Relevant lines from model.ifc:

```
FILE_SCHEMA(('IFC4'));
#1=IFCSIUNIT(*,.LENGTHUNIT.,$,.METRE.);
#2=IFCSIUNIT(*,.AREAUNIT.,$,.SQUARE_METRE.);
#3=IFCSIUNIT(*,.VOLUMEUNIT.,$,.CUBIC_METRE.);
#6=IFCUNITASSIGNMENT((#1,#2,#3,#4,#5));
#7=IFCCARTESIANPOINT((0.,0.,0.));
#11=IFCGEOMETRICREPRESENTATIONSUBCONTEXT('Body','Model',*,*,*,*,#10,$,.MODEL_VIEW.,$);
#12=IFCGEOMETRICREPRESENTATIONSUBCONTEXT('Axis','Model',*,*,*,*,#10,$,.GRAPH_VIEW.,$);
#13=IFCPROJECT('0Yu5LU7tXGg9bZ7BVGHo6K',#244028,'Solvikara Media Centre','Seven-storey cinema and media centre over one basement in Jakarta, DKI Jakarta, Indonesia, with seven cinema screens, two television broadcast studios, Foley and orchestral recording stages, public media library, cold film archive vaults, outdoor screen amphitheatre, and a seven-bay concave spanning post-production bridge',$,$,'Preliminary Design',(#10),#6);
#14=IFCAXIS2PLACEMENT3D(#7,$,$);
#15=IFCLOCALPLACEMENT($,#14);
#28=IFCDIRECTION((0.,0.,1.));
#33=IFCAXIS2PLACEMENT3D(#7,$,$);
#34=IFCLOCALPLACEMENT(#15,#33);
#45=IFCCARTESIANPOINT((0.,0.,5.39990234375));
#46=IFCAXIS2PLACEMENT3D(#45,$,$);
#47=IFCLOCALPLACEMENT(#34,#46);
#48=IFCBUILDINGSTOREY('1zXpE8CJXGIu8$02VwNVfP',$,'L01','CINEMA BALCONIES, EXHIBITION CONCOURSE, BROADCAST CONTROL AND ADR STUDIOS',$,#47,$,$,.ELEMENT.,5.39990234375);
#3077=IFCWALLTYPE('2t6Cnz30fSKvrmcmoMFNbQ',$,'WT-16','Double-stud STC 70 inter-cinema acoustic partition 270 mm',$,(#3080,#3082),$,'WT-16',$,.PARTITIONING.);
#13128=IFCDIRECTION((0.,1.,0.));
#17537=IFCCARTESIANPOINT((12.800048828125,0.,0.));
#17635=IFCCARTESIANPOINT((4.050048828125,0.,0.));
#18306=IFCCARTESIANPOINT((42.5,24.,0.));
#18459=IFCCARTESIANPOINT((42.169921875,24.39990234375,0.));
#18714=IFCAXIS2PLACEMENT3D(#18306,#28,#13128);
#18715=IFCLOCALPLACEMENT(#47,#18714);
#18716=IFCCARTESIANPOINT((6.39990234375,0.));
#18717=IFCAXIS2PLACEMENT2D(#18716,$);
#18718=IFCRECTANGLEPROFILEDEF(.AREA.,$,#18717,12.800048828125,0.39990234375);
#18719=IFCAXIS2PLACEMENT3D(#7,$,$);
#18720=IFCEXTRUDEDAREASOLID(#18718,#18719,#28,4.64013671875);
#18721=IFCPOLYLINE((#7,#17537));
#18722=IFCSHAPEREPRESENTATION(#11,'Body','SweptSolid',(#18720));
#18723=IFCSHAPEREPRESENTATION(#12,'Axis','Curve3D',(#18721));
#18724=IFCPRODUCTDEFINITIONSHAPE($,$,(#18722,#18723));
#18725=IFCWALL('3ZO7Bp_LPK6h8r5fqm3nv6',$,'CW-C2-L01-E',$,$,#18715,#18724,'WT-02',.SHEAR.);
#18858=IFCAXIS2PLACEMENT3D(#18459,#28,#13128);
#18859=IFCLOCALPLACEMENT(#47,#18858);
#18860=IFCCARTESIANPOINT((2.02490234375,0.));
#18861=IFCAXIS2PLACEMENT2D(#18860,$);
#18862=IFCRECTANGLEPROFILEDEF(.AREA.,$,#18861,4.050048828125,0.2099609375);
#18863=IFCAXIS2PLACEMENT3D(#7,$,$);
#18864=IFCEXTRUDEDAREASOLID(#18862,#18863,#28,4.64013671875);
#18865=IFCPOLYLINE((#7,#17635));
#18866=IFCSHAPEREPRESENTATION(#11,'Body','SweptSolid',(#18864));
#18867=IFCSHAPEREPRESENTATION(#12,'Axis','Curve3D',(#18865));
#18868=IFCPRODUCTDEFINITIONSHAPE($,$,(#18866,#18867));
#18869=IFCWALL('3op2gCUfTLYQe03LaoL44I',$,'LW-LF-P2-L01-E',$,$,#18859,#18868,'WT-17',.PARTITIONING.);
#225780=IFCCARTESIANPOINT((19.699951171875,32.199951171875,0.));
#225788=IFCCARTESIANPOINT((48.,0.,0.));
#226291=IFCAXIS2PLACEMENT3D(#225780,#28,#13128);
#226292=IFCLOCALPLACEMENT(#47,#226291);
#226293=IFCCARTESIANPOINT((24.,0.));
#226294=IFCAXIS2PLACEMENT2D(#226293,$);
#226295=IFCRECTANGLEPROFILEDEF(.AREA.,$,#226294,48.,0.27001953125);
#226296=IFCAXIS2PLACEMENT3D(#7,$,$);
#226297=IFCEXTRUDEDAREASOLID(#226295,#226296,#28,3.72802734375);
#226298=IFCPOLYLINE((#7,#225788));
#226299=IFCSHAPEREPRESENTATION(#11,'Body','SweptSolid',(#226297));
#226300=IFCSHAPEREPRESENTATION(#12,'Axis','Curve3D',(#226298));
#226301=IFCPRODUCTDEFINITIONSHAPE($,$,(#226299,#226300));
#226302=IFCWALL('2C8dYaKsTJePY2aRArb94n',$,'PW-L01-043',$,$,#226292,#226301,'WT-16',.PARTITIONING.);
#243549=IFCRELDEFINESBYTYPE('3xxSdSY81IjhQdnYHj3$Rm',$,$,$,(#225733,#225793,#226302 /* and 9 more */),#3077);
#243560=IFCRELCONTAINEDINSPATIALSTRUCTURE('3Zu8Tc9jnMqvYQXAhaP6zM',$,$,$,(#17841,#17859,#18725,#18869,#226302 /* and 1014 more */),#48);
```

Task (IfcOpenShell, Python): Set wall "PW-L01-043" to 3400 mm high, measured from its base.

```python
import ifcopenshell
import ifcopenshell.geom
import ifcopenshell.util.representation
import ifcopenshell.util.shape
import ifcopenshell.util.unit

model = ifcopenshell.open("model.ifc")
unit_scale = ifcopenshell.util.unit.calculate_unit_scale(model)
settings = ifcopenshell.geom.settings()


def volume(element):
    """Net volume in cubic metres, openings subtracted."""
    shape = ifcopenshell.geom.create_shape(settings, element)
    return ifcopenshell.util.shape.get_volume(shape.geometry)


wall = model.by_guid("2C8dYaKsTJePY2aRArb94n")
before = volume(wall)

body = ifcopenshell.util.representation.get_representation(wall, "Model", "Body")
solid = body.Items[0]
old_height = solid.Depth
solid.Depth = 3.4 / unit_scale
after = volume(wall)

print(f"height {old_height:g} -> {solid.Depth:g}, volume {before:.3f} -> {after:.3f} m3")

model.write("model-out.ifc")
```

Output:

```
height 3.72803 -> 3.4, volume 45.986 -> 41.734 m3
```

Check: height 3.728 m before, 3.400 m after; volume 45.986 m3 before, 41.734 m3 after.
